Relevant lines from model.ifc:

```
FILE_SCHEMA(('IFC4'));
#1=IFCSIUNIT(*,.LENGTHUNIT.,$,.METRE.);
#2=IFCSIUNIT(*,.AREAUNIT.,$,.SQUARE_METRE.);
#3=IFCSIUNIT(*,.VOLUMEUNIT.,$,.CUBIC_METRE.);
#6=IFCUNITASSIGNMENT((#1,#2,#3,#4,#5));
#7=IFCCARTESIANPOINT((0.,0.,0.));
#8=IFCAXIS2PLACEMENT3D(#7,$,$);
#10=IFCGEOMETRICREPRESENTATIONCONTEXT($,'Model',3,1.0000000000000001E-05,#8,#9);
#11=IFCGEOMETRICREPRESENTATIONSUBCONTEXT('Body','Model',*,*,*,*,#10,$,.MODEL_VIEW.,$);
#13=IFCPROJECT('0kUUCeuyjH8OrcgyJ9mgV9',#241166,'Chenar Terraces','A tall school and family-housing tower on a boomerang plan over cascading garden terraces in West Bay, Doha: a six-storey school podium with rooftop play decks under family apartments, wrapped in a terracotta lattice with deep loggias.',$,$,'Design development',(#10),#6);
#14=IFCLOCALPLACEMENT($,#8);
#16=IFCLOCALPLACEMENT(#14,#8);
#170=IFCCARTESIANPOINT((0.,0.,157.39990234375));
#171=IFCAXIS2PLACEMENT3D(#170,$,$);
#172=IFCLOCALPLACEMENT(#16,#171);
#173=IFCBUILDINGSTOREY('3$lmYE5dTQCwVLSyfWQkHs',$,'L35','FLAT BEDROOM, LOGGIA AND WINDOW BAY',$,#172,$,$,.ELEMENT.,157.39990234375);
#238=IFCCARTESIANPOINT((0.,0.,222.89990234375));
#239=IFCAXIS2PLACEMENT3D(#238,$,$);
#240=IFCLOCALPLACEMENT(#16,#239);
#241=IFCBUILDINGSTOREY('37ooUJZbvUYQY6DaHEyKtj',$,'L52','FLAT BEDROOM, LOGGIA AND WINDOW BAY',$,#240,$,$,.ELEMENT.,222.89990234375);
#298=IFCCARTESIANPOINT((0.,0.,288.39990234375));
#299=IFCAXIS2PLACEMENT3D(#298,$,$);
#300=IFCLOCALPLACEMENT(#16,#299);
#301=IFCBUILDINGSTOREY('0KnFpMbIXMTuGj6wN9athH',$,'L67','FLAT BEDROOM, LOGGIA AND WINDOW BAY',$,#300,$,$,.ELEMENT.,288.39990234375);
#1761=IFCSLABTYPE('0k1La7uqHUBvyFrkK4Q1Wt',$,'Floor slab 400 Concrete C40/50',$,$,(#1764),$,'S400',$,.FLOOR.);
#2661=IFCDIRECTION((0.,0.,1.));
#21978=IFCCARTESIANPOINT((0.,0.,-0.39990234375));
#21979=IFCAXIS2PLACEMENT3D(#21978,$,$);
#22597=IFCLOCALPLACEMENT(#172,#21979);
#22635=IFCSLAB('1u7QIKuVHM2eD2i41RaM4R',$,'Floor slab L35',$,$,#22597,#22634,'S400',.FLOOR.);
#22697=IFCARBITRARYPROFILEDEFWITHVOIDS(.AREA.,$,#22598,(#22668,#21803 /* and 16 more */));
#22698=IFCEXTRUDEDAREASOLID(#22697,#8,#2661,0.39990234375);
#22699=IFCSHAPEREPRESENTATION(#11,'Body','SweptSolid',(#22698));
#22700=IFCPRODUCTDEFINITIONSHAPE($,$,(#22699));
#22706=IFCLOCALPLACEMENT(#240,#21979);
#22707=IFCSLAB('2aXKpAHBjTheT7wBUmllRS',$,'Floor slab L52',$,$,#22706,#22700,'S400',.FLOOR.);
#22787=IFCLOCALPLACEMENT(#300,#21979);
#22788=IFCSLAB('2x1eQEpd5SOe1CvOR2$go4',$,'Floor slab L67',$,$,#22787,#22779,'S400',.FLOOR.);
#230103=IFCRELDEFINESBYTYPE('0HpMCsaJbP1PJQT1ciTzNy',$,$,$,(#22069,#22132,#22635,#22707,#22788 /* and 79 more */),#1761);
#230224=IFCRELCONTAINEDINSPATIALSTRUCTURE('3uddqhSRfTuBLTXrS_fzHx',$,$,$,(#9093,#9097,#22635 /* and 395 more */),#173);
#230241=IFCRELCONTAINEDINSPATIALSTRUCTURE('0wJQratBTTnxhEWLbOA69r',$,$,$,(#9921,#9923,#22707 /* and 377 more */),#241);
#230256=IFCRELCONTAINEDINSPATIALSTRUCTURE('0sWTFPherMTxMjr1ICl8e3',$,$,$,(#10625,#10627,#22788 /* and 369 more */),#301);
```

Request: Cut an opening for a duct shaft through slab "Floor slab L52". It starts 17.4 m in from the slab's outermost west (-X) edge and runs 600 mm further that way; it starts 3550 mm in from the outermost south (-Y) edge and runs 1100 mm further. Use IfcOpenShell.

```python
import numpy as np
import ifcopenshell
import ifcopenshell.api.feature
import ifcopenshell.api.geometry
import ifcopenshell.api.root
import ifcopenshell.geom
import ifcopenshell.util.placement
import ifcopenshell.util.representation
import ifcopenshell.util.shape
import ifcopenshell.util.unit

model = ifcopenshell.open("model.ifc")
unit_scale = ifcopenshell.util.unit.calculate_unit_scale(model)
settings = ifcopenshell.geom.settings()


def volume(element):
    """Net volume in cubic metres, openings subtracted."""
    shape = ifcopenshell.geom.create_shape(settings, element)
    return ifcopenshell.util.shape.get_volume(shape.geometry)


slab = model.by_guid("2aXKpAHBjTheT7wBUmllRS")
before = volume(slab)

# Extent in the slab's own axes, in metres. The edges named are its -X and -Y sides.
slab_shape = ifcopenshell.geom.create_shape(settings, slab)
vertices = ifcopenshell.util.shape.get_vertices(slab_shape.geometry)
x_min, y_min, bottom = vertices.min(axis=0)
top = vertices[:, 2].max()

opening = ifcopenshell.api.root.create_entity(model, ifc_class="IfcOpeningElement", name="Duct shaft opening", predefined_type="OPENING")
context = ifcopenshell.util.representation.get_context(model, "Model", "Body", "MODEL_VIEW")
width, depth = 0.6, 1.1
outline = [(0.0, 0.0), (width, 0.0), (width, depth), (0.0, depth), (0.0, 0.0)]
# Overshoot both faces by 50 mm so the cut is clean.
shape = ifcopenshell.api.geometry.add_slab_representation(
    model, context=context, depth=top - bottom + 0.1, polyline=outline
)
ifcopenshell.api.geometry.assign_representation(model, product=opening, representation=shape)

matrix = ifcopenshell.util.placement.get_local_placement(slab.ObjectPlacement)
matrix[:, 3] = matrix @ np.append(np.array([x_min + 17.4, y_min + 3.55, bottom - 0.05]) / unit_scale, 1.0)
ifcopenshell.api.geometry.edit_object_placement(model, product=opening, matrix=matrix, is_si=False)
ifcopenshell.api.feature.add_feature(model, feature=opening, element=slab)

after = volume(slab)

print(f"slab volume {before:.3f} -> {after:.3f} m3")

model.write("model_updated.ifc")
```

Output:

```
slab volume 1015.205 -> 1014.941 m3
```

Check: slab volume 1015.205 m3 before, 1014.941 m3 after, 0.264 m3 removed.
